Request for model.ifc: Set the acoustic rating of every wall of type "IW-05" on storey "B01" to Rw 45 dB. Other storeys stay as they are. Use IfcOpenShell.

First a look at what the model holds.

```python
import ifcopenshell
import ifcopenshell.util.element

model = ifcopenshell.open("model.ifc")
print(model.schema)
storey = next(s for s in model.by_type("IfcBuildingStorey") if s.Name == "B01")
walls = [e for e in ifcopenshell.util.element.get_decomposition(storey) if e.is_a("IfcWall")]
seen = {}
for e in walls:
    element_type = ifcopenshell.util.element.get_type(e)
    key = (element_type.Name if element_type != e and element_type else None, ifcopenshell.util.element.get_pset(e, "Pset_WallCommon", "AcousticRating"))
    seen[key] = seen.get(key, 0) + 1
for (name, value), count in sorted(seen.items(), key=str):
    print(count, "x", name, "|", value)
```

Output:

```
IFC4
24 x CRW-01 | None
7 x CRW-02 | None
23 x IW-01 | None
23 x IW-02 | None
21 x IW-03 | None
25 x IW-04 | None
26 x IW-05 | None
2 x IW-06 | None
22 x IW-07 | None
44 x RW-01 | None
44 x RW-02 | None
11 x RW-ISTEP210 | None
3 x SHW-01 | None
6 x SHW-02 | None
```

```python
import ifcopenshell
import ifcopenshell.api.pset
import ifcopenshell.util.element

model = ifcopenshell.open("model.ifc")

storey = next(s for s in model.by_type("IfcBuildingStorey") if s.Name == "B01")
walls = [e for e in ifcopenshell.util.element.get_decomposition(storey) if e.is_a("IfcWall")]

count = 0
for e in walls:
    element_type = ifcopenshell.util.element.get_type(e)
    if element_type in (None, e) or element_type.Name != "IW-05":
        continue
    # add_pset returns the element's existing set when there is one.
    pset = ifcopenshell.api.pset.add_pset(model, product=e, name="Pset_WallCommon")
    ifcopenshell.api.pset.edit_pset(model, pset=pset, properties={"AcousticRating": "Rw 45 dB"})
    count += 1

print(count, "walls updated")

model.write("model-out.ifc")
```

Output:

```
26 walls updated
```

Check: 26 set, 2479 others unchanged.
